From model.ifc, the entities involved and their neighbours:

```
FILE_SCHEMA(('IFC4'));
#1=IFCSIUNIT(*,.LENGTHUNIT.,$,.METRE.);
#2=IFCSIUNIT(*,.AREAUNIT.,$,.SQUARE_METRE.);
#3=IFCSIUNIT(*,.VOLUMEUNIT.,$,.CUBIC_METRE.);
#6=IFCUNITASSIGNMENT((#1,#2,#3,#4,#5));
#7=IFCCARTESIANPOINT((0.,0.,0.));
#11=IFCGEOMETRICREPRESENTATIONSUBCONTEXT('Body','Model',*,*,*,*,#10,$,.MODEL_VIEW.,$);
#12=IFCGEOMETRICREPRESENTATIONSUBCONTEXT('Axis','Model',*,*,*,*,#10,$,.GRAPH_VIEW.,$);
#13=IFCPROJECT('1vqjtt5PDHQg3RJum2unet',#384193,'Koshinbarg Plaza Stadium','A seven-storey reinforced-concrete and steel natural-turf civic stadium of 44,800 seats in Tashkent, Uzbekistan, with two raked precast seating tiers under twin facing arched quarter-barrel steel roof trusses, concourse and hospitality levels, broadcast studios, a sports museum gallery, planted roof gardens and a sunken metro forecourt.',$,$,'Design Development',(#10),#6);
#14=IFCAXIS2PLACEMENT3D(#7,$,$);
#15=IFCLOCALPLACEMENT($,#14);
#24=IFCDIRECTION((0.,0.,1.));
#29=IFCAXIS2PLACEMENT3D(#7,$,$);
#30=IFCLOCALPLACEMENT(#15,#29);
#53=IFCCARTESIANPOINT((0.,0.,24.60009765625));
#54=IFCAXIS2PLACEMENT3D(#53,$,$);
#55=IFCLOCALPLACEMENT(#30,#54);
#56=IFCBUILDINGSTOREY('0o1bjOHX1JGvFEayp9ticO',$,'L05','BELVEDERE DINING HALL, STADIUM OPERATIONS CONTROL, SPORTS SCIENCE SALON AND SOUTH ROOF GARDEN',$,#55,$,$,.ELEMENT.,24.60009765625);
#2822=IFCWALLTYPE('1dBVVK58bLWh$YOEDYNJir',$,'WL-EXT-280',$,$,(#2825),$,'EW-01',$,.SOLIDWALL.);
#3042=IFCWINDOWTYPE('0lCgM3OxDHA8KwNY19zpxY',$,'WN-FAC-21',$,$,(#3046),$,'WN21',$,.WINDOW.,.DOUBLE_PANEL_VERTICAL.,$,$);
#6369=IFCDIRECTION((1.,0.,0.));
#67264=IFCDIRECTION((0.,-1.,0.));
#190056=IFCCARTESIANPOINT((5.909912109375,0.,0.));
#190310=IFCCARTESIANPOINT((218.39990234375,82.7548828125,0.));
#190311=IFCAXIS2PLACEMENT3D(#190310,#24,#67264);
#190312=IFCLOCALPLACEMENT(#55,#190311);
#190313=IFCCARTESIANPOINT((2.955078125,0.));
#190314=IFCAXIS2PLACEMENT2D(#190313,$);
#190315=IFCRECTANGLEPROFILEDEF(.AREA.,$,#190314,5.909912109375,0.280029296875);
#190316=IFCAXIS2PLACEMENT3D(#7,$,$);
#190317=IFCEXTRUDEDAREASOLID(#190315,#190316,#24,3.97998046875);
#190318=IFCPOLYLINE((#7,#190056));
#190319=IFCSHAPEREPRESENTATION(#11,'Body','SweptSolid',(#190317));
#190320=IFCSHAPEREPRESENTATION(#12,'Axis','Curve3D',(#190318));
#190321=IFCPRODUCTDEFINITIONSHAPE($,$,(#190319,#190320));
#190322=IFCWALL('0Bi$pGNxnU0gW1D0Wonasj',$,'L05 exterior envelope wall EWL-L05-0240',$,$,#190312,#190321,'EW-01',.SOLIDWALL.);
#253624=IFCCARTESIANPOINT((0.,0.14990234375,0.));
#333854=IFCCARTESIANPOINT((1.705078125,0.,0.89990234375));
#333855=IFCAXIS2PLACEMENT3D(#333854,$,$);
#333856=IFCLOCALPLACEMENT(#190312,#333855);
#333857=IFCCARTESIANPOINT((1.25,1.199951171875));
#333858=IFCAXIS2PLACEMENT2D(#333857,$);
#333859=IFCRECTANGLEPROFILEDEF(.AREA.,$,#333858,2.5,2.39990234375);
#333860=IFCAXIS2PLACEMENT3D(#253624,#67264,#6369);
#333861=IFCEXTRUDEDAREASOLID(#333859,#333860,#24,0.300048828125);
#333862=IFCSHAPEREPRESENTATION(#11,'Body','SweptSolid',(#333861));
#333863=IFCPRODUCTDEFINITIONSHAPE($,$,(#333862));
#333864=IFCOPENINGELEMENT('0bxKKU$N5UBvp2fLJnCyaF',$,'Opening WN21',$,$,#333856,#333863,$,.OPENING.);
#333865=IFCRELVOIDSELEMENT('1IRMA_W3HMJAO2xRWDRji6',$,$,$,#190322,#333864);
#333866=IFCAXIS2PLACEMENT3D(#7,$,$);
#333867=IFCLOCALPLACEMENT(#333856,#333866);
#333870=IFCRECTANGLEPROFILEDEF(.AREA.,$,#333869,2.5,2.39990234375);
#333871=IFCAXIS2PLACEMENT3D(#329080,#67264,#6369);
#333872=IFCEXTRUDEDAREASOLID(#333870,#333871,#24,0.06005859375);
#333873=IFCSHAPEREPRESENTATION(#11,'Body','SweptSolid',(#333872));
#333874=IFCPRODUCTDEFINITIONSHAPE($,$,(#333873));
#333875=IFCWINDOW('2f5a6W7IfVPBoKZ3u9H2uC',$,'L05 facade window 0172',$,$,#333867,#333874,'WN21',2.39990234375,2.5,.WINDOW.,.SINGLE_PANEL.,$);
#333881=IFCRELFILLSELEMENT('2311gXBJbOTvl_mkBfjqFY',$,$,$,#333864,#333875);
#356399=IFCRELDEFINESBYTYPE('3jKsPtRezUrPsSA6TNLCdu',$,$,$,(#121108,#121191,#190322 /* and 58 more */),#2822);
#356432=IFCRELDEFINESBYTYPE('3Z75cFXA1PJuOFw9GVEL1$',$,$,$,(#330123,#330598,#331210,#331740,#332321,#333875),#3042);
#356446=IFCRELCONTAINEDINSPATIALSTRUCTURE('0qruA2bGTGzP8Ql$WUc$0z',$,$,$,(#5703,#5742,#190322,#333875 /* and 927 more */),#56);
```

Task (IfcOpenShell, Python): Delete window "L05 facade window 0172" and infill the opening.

```python
import ifcopenshell
import ifcopenshell.api.feature
import ifcopenshell.api.root
import ifcopenshell.geom
import ifcopenshell.util.shape

model = ifcopenshell.open("model.ifc")
settings = ifcopenshell.geom.settings()


def volume(element):
    """Net volume in cubic metres, openings subtracted."""
    shape = ifcopenshell.geom.create_shape(settings, element)
    return ifcopenshell.util.shape.get_volume(shape.geometry)


window = model.by_id(333875)
opening = window.FillsVoids[0].RelatingOpeningElement
wall = opening.VoidsElements[0].RelatingBuildingElement
before = volume(wall)

ifcopenshell.api.root.remove_product(model, product=window)
ifcopenshell.api.feature.remove_feature(model, feature=opening)

after = volume(wall)

print(f"wall volume {before:.3f} -> {after:.3f} m3")

model.write("model_rev.ifc")
```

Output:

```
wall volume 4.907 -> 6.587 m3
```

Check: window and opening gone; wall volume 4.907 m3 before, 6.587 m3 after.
